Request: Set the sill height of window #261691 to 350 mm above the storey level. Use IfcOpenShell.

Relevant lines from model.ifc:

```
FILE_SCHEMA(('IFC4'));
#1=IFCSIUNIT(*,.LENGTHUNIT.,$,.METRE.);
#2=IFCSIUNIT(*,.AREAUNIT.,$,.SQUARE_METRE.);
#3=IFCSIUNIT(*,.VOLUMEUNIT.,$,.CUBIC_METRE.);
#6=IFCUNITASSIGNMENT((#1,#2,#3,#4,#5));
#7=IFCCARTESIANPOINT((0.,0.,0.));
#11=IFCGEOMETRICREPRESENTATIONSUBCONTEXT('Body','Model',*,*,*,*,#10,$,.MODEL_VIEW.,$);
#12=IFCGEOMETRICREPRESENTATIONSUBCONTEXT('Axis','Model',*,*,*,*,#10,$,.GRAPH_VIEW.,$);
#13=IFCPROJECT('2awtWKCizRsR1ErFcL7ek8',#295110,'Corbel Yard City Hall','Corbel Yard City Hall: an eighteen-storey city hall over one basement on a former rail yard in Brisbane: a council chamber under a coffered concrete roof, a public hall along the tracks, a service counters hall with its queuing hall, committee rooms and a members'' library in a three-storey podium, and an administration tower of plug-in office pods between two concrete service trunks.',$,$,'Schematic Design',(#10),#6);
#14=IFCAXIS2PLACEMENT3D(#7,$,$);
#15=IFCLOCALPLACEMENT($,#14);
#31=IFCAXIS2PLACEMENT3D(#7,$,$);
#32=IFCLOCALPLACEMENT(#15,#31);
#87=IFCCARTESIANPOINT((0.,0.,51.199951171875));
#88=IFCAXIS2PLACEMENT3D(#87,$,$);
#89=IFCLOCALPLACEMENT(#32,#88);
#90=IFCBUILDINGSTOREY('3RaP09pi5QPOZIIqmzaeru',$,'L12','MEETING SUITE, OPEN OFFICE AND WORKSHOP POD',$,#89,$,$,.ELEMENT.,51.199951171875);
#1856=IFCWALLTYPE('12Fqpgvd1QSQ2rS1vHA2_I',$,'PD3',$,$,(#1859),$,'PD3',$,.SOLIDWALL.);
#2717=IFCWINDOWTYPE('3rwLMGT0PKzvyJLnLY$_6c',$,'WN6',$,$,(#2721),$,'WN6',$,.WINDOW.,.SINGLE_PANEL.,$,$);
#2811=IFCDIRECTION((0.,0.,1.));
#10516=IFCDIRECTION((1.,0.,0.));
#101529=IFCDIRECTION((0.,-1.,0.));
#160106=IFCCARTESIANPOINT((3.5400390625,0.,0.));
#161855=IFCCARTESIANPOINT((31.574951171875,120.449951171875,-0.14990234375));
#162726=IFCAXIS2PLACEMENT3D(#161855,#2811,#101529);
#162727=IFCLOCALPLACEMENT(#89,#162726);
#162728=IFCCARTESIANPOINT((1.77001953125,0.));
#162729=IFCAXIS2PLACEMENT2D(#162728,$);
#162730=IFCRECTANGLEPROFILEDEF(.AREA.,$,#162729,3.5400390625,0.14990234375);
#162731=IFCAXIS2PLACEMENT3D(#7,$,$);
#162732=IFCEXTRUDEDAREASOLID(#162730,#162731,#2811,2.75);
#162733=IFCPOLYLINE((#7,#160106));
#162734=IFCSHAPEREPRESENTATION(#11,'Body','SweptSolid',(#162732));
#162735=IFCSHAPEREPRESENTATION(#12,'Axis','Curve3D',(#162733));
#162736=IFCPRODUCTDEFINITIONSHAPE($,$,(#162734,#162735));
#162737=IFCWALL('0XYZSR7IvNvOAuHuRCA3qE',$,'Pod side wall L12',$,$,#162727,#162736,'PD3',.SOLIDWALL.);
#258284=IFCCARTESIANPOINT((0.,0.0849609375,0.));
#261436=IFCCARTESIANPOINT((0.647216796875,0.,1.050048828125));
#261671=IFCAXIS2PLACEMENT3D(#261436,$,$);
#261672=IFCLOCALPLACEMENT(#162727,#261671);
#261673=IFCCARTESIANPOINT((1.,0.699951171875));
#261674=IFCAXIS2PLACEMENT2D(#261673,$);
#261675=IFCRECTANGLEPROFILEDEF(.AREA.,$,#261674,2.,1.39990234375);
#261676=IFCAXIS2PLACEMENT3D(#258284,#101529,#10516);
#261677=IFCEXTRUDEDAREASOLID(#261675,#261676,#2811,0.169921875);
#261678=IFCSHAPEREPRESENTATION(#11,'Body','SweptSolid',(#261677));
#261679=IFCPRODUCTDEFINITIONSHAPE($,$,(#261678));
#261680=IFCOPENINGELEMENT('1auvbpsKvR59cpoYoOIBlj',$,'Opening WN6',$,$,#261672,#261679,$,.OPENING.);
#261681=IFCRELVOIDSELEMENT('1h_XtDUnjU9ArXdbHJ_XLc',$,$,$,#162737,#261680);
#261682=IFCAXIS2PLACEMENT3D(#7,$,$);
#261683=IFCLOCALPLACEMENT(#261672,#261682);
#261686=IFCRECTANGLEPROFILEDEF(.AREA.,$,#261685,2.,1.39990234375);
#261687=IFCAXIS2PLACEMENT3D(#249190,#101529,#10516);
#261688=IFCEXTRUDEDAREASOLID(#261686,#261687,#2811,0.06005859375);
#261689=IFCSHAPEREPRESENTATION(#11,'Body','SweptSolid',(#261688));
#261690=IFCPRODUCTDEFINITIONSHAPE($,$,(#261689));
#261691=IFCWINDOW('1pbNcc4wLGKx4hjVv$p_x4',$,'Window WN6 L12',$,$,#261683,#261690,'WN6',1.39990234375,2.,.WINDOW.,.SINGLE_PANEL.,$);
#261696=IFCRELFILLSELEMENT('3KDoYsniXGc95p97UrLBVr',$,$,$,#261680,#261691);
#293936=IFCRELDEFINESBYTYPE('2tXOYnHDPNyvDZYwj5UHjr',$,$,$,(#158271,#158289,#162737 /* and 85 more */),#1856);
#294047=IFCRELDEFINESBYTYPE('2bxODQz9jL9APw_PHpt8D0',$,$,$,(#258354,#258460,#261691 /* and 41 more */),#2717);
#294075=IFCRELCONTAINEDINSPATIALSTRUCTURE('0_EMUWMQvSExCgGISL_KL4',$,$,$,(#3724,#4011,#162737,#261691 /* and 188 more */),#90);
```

```python
import numpy as np
import ifcopenshell
import ifcopenshell.api.geometry
import ifcopenshell.geom
import ifcopenshell.util.element
import ifcopenshell.util.placement
import ifcopenshell.util.shape
import ifcopenshell.util.unit

model = ifcopenshell.open("model.ifc")
unit_scale = ifcopenshell.util.unit.calculate_unit_scale(model)

window = model.by_guid("1pbNcc4wLGKx4hjVv$p_x4")
opening = window.FillsVoids[0].RelatingOpeningElement
storey = ifcopenshell.util.element.get_container(window, ifc_class="IfcBuildingStorey")
level = ifcopenshell.util.placement.get_local_placement(storey.ObjectPlacement)[2, 3]

# The opening's origin need not be at the sill, so measure its lowest point.
shape = ifcopenshell.geom.create_shape(ifcopenshell.geom.settings(), opening)
bottom = ifcopenshell.util.shape.get_shape_bottom_elevation(shape, shape.geometry) / unit_scale
dz = level + 0.35 / unit_scale - bottom

shift = np.array([0.0, 0.0, dz])
# The window is placed relative to its opening, so it follows when the opening moves.
matrix = ifcopenshell.util.placement.get_local_placement(opening.ObjectPlacement)
matrix[:3, 3] += shift
ifcopenshell.api.geometry.edit_object_placement(
    model, product=opening, matrix=matrix, is_si=False, should_transform_children=True
)

print(f"moved by {dz * unit_scale:+.3f} m")

model.write("model_rev.ifc")
```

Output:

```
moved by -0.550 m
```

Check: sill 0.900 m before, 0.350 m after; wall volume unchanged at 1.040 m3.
